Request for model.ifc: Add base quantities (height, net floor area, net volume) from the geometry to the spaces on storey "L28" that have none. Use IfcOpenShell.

First a look at what the model holds.

```python
import ifcopenshell
import ifcopenshell.util.element
import ifcopenshell.util.unit

model = ifcopenshell.open("model.ifc")
print(model.schema)
for unit_type in ("LENGTHUNIT", "AREAUNIT", "VOLUMEUNIT"):
    print(unit_type, ifcopenshell.util.unit.calculate_unit_scale(model, unit_type))
storey = next(s for s in model.by_type("IfcBuildingStorey") if s.Name == "L28")
spaces = [e for e in ifcopenshell.util.element.get_decomposition(storey) if e.is_a("IfcSpace")]
for e in sorted(spaces, key=lambda e: e.id()):
    print(e.id(), e.is_a(), e.Name, list(ifcopenshell.util.element.get_psets(e, qtos_only=True)), sep=" | ")
```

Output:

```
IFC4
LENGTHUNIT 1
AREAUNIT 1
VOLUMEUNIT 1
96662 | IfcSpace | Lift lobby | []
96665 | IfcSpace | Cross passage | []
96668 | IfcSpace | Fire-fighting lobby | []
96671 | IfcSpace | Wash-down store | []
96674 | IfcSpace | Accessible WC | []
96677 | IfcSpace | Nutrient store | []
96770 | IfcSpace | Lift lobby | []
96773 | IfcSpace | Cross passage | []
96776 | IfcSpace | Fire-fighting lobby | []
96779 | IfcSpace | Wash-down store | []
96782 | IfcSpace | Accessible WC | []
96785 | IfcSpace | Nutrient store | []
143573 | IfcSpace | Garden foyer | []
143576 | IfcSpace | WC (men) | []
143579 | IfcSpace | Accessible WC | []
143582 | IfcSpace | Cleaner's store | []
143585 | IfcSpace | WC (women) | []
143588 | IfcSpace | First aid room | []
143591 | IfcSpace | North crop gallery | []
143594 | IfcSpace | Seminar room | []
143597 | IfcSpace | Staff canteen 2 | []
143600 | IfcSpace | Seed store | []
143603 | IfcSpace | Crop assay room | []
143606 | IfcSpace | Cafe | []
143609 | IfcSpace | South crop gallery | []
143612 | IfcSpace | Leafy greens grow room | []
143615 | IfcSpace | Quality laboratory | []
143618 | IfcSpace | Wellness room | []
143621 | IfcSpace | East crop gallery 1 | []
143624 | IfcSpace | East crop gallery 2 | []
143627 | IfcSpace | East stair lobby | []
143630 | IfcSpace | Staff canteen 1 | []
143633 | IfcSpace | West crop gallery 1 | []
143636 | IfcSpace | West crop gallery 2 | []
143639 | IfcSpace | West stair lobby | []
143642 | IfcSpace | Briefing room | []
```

```python
import ifcopenshell
import ifcopenshell.api.pset
import ifcopenshell.geom
import ifcopenshell.util.element
import ifcopenshell.util.shape
import ifcopenshell.util.unit

model = ifcopenshell.open("model.ifc")
unit_scale = ifcopenshell.util.unit.calculate_unit_scale(model)
area_scale = ifcopenshell.util.unit.calculate_unit_scale(model, "AREAUNIT")
volume_scale = ifcopenshell.util.unit.calculate_unit_scale(model, "VOLUMEUNIT")
settings = ifcopenshell.geom.settings()

storey = next(s for s in model.by_type("IfcBuildingStorey") if s.Name == "L28")
spaces = [e for e in ifcopenshell.util.element.get_decomposition(storey) if e.is_a("IfcSpace")]

for e in sorted(spaces, key=lambda e: e.id()):
    if ifcopenshell.util.element.get_psets(e, qtos_only=True, should_inherit=False):
        continue
    # Geometry comes back in metres, in the element's own axes.
    shape = ifcopenshell.geom.create_shape(settings, e)
    values = {
        "Height": ifcopenshell.util.shape.get_z(shape.geometry) / unit_scale,
        "NetFloorArea": ifcopenshell.util.shape.get_footprint_area(shape.geometry) / area_scale,
        "NetVolume": ifcopenshell.util.shape.get_volume(shape.geometry) / volume_scale,
    }
    qto = ifcopenshell.api.pset.add_qto(model, product=e, name="Qto_SpaceBaseQuantities")
    ifcopenshell.api.pset.edit_qto(model, qto=qto, properties=values)
    print(e.id(), {k: round(v, 3) for k, v in values.items()})

model.write("model_rev.ifc")
```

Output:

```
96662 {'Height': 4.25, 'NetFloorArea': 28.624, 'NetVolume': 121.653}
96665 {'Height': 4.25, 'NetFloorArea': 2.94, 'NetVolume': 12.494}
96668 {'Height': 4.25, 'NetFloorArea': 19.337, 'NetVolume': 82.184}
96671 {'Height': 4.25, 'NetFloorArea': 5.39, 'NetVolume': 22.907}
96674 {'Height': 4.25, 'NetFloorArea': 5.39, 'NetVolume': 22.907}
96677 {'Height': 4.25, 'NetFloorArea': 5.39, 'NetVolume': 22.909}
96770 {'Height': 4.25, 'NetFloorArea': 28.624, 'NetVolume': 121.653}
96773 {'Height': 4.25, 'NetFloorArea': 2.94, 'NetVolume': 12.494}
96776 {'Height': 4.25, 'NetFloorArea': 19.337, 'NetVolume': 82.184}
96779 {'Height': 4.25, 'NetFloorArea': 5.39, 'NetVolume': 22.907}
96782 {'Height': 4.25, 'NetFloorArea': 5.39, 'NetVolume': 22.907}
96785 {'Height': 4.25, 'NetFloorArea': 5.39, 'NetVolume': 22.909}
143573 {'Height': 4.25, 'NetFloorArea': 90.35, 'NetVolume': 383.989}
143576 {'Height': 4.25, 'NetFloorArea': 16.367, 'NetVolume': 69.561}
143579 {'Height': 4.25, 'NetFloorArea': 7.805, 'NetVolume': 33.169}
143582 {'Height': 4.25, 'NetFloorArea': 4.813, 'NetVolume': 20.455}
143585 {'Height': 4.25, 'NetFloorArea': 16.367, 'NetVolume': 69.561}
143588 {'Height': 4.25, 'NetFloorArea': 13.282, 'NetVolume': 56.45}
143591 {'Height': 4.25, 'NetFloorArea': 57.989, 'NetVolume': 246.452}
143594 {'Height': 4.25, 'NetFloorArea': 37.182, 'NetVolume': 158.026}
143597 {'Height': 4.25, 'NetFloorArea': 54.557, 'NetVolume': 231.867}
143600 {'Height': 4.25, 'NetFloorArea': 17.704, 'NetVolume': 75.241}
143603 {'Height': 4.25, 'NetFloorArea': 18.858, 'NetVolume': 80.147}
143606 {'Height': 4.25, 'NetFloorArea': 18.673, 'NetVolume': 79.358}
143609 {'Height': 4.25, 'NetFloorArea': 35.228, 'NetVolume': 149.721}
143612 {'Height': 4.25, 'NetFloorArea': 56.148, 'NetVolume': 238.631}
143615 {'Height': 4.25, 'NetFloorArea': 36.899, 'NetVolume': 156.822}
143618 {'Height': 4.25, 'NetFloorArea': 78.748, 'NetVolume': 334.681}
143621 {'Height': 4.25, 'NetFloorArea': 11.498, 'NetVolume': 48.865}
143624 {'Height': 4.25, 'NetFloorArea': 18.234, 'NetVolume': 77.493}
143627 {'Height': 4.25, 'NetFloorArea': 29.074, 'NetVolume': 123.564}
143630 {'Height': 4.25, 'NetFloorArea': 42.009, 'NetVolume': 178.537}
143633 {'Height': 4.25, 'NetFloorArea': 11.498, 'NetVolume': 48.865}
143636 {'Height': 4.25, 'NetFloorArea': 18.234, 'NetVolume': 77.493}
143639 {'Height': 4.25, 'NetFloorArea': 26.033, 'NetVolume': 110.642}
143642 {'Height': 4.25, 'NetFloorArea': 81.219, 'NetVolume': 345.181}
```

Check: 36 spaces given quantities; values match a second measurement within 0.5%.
